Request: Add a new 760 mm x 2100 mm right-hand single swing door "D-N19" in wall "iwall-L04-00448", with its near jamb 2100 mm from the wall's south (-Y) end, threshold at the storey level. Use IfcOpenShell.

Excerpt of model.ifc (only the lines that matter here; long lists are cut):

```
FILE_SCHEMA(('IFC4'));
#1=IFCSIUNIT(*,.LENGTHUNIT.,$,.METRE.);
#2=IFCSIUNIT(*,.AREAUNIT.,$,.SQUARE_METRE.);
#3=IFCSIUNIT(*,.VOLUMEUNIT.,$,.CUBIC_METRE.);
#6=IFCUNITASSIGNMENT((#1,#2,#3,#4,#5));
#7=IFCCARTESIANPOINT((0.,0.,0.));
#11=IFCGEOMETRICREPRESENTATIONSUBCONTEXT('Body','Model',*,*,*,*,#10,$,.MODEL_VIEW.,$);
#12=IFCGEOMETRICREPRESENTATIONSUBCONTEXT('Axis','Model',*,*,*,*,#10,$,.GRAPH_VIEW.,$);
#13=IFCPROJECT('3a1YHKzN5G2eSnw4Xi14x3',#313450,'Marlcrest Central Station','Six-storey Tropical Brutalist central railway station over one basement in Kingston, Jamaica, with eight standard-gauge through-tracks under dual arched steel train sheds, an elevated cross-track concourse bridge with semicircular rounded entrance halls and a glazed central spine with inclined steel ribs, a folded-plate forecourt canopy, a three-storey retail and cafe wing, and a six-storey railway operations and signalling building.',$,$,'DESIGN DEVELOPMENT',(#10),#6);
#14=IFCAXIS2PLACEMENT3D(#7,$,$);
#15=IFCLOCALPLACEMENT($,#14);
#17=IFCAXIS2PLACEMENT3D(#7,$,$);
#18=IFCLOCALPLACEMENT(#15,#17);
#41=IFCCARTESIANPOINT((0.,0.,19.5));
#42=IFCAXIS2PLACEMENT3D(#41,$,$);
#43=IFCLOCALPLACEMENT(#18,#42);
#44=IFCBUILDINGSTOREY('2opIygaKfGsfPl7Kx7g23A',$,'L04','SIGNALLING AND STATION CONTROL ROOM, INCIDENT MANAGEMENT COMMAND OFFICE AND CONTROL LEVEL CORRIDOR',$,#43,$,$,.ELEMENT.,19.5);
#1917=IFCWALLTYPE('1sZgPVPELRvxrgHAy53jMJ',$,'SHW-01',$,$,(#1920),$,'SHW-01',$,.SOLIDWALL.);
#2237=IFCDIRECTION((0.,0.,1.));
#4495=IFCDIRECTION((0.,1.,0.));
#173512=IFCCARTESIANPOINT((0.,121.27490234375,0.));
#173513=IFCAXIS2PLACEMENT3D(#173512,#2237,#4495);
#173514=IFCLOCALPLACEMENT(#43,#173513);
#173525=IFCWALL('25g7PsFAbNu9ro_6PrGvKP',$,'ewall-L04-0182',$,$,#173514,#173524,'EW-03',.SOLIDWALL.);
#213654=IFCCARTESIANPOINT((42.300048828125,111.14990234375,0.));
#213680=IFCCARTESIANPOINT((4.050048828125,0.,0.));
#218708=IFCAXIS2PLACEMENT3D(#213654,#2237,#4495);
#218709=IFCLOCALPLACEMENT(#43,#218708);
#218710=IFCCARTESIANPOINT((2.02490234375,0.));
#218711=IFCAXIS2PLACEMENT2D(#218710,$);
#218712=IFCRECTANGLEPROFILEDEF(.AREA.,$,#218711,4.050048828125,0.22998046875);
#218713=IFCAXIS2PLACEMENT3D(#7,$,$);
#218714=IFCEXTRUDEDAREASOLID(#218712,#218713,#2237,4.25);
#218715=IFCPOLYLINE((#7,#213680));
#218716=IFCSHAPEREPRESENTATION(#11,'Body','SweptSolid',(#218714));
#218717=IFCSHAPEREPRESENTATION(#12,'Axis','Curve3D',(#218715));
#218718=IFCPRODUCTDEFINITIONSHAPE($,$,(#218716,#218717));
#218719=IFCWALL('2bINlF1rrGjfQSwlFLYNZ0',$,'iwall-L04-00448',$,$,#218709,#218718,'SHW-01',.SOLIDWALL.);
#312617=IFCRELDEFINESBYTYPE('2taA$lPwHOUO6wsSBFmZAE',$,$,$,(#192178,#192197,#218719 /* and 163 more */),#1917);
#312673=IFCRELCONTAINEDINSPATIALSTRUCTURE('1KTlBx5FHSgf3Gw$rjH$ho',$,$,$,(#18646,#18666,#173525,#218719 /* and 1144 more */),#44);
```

```python
import numpy as np
import ifcopenshell
import ifcopenshell.api.feature
import ifcopenshell.api.geometry
import ifcopenshell.api.root
import ifcopenshell.api.spatial
import ifcopenshell.geom
import ifcopenshell.util.element
import ifcopenshell.util.placement
import ifcopenshell.util.representation
import ifcopenshell.util.shape
import ifcopenshell.util.unit

model = ifcopenshell.open("model.ifc")
unit_scale = ifcopenshell.util.unit.calculate_unit_scale(model)
settings = ifcopenshell.geom.settings()


def volume(element):
    """Net volume in cubic metres, openings subtracted."""
    shape = ifcopenshell.geom.create_shape(settings, element)
    return ifcopenshell.util.shape.get_volume(shape.geometry)


wall = model.by_guid("2bINlF1rrGjfQSwlFLYNZ0")
storey = ifcopenshell.util.element.get_container(wall, ifc_class="IfcBuildingStorey")
context = ifcopenshell.util.representation.get_context(model, "Model", "Body", "MODEL_VIEW")
before = volume(wall)

width, height, from_end, sill = 0.76, 2.1, 2.1, 0.0  # metres

# The wall runs along its own X axis, and the end named is its -X end.
wall_shape = ifcopenshell.geom.create_shape(settings, wall)
x, y, z = ifcopenshell.util.shape.get_vertices(wall_shape.geometry).T
start = x.min() + from_end
face, thickness = float(y.min()), float(y.max() - y.min())
wall_matrix = ifcopenshell.util.placement.get_local_placement(wall.ObjectPlacement)
level = ifcopenshell.util.placement.get_local_placement(storey.ObjectPlacement)[2, 3]


def in_wall(x, y):
    """Placement at x, y metres in the wall's axes, at sill height."""
    matrix = wall_matrix.copy()
    matrix[:, 3] = wall_matrix @ np.array([x / unit_scale, y / unit_scale, 0.0, 1.0])
    matrix[2, 3] = level + sill / unit_scale
    return matrix


# Opening: a box that overshoots both wall faces by 50 mm.
opening = ifcopenshell.api.root.create_entity(model, ifc_class="IfcOpeningElement", predefined_type="OPENING")
box = ifcopenshell.api.geometry.add_wall_representation(
    model, context=context, length=width, height=height, thickness=thickness + 0.1
)
ifcopenshell.api.geometry.assign_representation(model, product=opening, representation=box)
ifcopenshell.api.geometry.edit_object_placement(model, product=opening, matrix=in_wall(start, face - 0.05), is_si=False)
ifcopenshell.api.feature.add_feature(model, feature=opening, element=wall)

door = ifcopenshell.api.root.create_entity(model, ifc_class="IfcDoor", name="D-N19", predefined_type="DOOR")
door.OverallWidth, door.OverallHeight = width / unit_scale, height / unit_scale
door.OperationType = "SINGLE_SWING_RIGHT"
body = ifcopenshell.api.geometry.add_door_representation(
    model,
    context=context,
    overall_width=door.OverallWidth,
    overall_height=door.OverallHeight,
    operation_type="SINGLE_SWING_RIGHT",
    lining_properties={"LiningDepth": thickness / unit_scale, "ThresholdDepth": thickness / unit_scale},
)
ifcopenshell.api.geometry.assign_representation(model, product=door, representation=body)
ifcopenshell.api.spatial.assign_container(model, products=[door], relating_structure=storey)
ifcopenshell.api.feature.add_filling(model, opening=opening, element=door)

# The lining spans the wall, so the door starts at the wall face.
ifcopenshell.api.geometry.edit_object_placement(model, product=door, matrix=in_wall(start, face), is_si=False)

after = volume(wall)

print(f"wall volume {before:.3f} -> {after:.3f} m3")

model.write("model_v2.ifc")
```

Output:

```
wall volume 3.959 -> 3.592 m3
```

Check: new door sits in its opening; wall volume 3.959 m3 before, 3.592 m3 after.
